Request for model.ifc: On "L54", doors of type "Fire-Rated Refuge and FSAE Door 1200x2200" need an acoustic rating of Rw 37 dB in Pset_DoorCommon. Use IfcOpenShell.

First a look at what the model holds.

```python
import ifcopenshell
import ifcopenshell.util.element

model = ifcopenshell.open("model.ifc")
print(model.schema)
storey = next(s for s in model.by_type("IfcBuildingStorey") if s.Name == "L54")
doors = [e for e in ifcopenshell.util.element.get_decomposition(storey) if e.is_a("IfcDoor")]
seen = {}
for e in doors:
    element_type = ifcopenshell.util.element.get_type(e)
    key = (element_type.Name if element_type != e and element_type else None, ifcopenshell.util.element.get_pset(e, "Pset_DoorCommon", "AcousticRating"))
    seen[key] = seen.get(key, 0) + 1
for (name, value), count in sorted(seen.items(), key=str):
    print(count, "x", name, "|", value)
```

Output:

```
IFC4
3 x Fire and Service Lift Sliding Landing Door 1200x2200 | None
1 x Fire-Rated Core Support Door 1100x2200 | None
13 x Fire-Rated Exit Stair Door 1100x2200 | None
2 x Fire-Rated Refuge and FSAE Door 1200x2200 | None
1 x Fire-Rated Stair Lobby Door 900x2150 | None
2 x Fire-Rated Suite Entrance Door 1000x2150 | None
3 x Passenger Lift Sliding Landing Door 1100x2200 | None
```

```python
import ifcopenshell
import ifcopenshell.api.pset
import ifcopenshell.util.element

model = ifcopenshell.open("model.ifc")

storey = next(s for s in model.by_type("IfcBuildingStorey") if s.Name == "L54")
doors = [e for e in ifcopenshell.util.element.get_decomposition(storey) if e.is_a("IfcDoor")]

count = 0
for e in doors:
    element_type = ifcopenshell.util.element.get_type(e)
    if element_type in (None, e) or element_type.Name != "Fire-Rated Refuge and FSAE Door 1200x2200":
        continue
    # add_pset returns the element's existing set when there is one.
    pset = ifcopenshell.api.pset.add_pset(model, product=e, name="Pset_DoorCommon")
    ifcopenshell.api.pset.edit_pset(model, pset=pset, properties={"AcousticRating": "Rw 37 dB"})
    count += 1

print(count, "doors updated")

model.write("model-out.ifc")
```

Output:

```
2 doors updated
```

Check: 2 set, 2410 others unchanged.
